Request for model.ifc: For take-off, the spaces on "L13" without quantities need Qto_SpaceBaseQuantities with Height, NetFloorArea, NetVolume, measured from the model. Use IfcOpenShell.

First a look at what the model holds.

```python
import ifcopenshell
import ifcopenshell.util.element
import ifcopenshell.util.unit

model = ifcopenshell.open("model.ifc")
print(model.schema)
for unit_type in ("LENGTHUNIT", "AREAUNIT", "VOLUMEUNIT"):
    print(unit_type, ifcopenshell.util.unit.calculate_unit_scale(model, unit_type))
storey = next(s for s in model.by_type("IfcBuildingStorey") if s.Name == "L13")
spaces = [e for e in ifcopenshell.util.element.get_decomposition(storey) if e.is_a("IfcSpace")]
for e in sorted(spaces, key=lambda e: e.id()):
    print(e.id(), e.is_a(), e.Name, list(ifcopenshell.util.element.get_psets(e, qtos_only=True)), sep=" | ")
```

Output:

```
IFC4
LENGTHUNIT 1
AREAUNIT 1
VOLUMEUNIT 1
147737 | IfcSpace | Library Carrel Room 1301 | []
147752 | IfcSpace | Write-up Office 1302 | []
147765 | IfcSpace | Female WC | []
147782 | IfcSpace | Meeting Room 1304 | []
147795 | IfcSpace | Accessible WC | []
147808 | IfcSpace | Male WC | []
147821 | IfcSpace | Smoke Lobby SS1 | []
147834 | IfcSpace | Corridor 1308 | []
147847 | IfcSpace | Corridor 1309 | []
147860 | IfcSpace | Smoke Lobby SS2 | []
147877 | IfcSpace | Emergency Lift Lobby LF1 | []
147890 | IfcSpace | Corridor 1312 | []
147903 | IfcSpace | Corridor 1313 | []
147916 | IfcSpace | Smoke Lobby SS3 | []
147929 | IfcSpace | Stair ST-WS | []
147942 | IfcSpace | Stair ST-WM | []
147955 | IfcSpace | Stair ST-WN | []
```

```python
import ifcopenshell
import ifcopenshell.api.pset
import ifcopenshell.geom
import ifcopenshell.util.element
import ifcopenshell.util.shape
import ifcopenshell.util.unit

model = ifcopenshell.open("model.ifc")
unit_scale = ifcopenshell.util.unit.calculate_unit_scale(model)
area_scale = ifcopenshell.util.unit.calculate_unit_scale(model, "AREAUNIT")
volume_scale = ifcopenshell.util.unit.calculate_unit_scale(model, "VOLUMEUNIT")
settings = ifcopenshell.geom.settings()

storey = next(s for s in model.by_type("IfcBuildingStorey") if s.Name == "L13")
spaces = [e for e in ifcopenshell.util.element.get_decomposition(storey) if e.is_a("IfcSpace")]

for e in sorted(spaces, key=lambda e: e.id()):
    if ifcopenshell.util.element.get_psets(e, qtos_only=True, should_inherit=False):
        continue
    # Geometry comes back in metres, in the element's own axes.
    shape = ifcopenshell.geom.create_shape(settings, e)
    values = {
        "Height": ifcopenshell.util.shape.get_z(shape.geometry) / unit_scale,
        "NetFloorArea": ifcopenshell.util.shape.get_footprint_area(shape.geometry) / area_scale,
        "NetVolume": ifcopenshell.util.shape.get_volume(shape.geometry) / volume_scale,
    }
    qto = ifcopenshell.api.pset.add_qto(model, product=e, name="Qto_SpaceBaseQuantities")
    ifcopenshell.api.pset.edit_qto(model, qto=qto, properties=values)
    print(e.id(), {k: round(v, 3) for k, v in values.items()})

model.write("model_v2.ifc")
```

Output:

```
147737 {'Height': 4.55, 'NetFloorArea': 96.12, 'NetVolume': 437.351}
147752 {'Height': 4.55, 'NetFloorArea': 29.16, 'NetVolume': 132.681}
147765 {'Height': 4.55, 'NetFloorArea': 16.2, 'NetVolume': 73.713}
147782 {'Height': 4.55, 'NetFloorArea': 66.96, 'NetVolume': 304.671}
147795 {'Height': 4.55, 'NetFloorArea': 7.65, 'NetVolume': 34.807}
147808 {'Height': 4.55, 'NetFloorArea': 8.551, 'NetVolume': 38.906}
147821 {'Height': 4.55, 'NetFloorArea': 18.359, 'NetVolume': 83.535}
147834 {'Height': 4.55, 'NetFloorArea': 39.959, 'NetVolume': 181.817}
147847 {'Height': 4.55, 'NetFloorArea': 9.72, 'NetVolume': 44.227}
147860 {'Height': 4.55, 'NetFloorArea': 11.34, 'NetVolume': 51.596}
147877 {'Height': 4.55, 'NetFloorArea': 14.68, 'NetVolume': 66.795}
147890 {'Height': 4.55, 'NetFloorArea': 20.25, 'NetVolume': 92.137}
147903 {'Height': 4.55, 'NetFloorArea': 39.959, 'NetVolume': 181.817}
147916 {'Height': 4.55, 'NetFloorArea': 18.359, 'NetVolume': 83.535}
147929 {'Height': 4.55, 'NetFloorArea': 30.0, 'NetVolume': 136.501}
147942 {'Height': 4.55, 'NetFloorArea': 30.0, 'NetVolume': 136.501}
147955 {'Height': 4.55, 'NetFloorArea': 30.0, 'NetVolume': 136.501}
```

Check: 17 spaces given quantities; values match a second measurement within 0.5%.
